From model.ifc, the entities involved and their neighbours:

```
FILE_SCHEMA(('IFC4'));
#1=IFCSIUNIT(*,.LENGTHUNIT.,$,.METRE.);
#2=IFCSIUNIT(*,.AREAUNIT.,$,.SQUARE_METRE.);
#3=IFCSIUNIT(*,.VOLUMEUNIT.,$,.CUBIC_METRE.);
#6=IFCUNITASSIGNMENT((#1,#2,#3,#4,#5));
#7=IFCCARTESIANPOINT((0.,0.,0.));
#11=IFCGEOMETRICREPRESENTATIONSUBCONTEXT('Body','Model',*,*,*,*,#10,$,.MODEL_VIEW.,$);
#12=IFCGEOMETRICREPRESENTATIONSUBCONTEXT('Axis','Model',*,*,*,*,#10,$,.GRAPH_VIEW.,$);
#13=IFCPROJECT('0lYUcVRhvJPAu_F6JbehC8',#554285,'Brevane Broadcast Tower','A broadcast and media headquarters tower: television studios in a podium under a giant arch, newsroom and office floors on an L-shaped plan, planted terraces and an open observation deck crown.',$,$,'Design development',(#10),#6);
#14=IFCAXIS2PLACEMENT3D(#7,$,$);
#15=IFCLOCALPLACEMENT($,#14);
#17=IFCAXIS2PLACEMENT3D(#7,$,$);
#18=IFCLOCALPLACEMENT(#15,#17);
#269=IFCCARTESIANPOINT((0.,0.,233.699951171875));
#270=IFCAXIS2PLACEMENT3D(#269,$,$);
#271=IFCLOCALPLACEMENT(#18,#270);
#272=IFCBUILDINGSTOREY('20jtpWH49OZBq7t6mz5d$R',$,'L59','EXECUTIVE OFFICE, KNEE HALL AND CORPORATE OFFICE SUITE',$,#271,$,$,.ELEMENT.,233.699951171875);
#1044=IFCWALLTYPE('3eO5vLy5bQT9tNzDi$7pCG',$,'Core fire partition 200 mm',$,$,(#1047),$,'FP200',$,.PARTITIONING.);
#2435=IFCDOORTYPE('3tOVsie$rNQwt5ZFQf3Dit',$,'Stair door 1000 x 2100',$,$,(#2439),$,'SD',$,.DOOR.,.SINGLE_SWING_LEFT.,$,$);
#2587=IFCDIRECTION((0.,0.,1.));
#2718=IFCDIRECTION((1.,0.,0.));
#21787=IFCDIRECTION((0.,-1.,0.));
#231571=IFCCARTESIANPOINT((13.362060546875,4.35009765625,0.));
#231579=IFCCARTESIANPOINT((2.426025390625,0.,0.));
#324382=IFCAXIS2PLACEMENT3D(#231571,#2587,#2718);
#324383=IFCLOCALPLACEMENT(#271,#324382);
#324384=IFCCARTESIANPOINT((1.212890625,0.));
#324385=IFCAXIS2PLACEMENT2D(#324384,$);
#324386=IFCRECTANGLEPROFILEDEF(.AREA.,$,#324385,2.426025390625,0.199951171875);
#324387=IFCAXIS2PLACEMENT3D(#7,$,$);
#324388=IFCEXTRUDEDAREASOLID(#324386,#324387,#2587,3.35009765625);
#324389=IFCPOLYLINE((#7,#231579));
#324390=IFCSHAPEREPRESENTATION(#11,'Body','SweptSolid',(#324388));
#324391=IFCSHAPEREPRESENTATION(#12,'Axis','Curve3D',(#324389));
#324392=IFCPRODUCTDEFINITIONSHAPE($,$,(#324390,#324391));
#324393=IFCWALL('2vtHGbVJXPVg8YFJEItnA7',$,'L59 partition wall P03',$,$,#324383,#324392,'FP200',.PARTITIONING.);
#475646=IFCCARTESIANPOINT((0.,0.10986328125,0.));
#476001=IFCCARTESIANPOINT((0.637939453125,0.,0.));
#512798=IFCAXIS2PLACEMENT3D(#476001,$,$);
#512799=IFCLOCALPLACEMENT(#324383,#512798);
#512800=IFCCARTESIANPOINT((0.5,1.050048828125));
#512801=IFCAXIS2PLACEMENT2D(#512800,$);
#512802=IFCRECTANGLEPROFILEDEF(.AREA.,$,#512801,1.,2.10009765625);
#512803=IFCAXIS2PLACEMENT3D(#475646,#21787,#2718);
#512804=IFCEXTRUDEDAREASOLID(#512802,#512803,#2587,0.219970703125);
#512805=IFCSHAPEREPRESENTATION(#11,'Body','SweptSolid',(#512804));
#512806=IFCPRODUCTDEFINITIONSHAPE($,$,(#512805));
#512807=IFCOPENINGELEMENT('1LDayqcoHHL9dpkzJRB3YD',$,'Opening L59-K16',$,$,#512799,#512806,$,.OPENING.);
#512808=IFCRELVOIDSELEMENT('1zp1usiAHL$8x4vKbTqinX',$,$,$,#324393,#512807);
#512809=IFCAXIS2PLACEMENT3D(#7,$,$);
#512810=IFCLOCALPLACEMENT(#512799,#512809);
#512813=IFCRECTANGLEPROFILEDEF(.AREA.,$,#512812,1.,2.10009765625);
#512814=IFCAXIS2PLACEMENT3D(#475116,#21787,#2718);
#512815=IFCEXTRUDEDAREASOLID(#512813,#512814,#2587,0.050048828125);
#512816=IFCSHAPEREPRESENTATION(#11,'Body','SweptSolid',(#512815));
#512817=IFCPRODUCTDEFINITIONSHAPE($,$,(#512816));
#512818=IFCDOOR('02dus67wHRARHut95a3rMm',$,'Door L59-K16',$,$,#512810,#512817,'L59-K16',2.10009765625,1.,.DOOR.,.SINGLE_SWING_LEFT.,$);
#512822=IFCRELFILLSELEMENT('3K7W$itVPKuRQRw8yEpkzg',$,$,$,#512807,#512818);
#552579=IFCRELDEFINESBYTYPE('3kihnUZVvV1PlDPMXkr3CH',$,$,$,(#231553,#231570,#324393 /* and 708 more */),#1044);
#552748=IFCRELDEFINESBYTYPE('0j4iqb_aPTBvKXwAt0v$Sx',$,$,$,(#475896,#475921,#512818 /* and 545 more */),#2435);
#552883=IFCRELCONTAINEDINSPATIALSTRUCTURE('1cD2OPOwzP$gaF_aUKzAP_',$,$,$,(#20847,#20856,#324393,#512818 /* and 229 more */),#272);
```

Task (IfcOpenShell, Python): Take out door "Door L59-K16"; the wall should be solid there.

```python
import ifcopenshell
import ifcopenshell.api.feature
import ifcopenshell.api.root
import ifcopenshell.geom
import ifcopenshell.util.shape

model = ifcopenshell.open("model.ifc")
settings = ifcopenshell.geom.settings()


def volume(element):
    """Net volume in cubic metres, openings subtracted."""
    shape = ifcopenshell.geom.create_shape(settings, element)
    return ifcopenshell.util.shape.get_volume(shape.geometry)


door = model.by_guid("02dus67wHRARHut95a3rMm")
opening = door.FillsVoids[0].RelatingOpeningElement
wall = opening.VoidsElements[0].RelatingBuildingElement
before = volume(wall)

ifcopenshell.api.root.remove_product(model, product=door)
ifcopenshell.api.feature.remove_feature(model, feature=opening)

after = volume(wall)

print(f"wall volume {before:.3f} -> {after:.3f} m3")

model.write("model_updated.ifc")
```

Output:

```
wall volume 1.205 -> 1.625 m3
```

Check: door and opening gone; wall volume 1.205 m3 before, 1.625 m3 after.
